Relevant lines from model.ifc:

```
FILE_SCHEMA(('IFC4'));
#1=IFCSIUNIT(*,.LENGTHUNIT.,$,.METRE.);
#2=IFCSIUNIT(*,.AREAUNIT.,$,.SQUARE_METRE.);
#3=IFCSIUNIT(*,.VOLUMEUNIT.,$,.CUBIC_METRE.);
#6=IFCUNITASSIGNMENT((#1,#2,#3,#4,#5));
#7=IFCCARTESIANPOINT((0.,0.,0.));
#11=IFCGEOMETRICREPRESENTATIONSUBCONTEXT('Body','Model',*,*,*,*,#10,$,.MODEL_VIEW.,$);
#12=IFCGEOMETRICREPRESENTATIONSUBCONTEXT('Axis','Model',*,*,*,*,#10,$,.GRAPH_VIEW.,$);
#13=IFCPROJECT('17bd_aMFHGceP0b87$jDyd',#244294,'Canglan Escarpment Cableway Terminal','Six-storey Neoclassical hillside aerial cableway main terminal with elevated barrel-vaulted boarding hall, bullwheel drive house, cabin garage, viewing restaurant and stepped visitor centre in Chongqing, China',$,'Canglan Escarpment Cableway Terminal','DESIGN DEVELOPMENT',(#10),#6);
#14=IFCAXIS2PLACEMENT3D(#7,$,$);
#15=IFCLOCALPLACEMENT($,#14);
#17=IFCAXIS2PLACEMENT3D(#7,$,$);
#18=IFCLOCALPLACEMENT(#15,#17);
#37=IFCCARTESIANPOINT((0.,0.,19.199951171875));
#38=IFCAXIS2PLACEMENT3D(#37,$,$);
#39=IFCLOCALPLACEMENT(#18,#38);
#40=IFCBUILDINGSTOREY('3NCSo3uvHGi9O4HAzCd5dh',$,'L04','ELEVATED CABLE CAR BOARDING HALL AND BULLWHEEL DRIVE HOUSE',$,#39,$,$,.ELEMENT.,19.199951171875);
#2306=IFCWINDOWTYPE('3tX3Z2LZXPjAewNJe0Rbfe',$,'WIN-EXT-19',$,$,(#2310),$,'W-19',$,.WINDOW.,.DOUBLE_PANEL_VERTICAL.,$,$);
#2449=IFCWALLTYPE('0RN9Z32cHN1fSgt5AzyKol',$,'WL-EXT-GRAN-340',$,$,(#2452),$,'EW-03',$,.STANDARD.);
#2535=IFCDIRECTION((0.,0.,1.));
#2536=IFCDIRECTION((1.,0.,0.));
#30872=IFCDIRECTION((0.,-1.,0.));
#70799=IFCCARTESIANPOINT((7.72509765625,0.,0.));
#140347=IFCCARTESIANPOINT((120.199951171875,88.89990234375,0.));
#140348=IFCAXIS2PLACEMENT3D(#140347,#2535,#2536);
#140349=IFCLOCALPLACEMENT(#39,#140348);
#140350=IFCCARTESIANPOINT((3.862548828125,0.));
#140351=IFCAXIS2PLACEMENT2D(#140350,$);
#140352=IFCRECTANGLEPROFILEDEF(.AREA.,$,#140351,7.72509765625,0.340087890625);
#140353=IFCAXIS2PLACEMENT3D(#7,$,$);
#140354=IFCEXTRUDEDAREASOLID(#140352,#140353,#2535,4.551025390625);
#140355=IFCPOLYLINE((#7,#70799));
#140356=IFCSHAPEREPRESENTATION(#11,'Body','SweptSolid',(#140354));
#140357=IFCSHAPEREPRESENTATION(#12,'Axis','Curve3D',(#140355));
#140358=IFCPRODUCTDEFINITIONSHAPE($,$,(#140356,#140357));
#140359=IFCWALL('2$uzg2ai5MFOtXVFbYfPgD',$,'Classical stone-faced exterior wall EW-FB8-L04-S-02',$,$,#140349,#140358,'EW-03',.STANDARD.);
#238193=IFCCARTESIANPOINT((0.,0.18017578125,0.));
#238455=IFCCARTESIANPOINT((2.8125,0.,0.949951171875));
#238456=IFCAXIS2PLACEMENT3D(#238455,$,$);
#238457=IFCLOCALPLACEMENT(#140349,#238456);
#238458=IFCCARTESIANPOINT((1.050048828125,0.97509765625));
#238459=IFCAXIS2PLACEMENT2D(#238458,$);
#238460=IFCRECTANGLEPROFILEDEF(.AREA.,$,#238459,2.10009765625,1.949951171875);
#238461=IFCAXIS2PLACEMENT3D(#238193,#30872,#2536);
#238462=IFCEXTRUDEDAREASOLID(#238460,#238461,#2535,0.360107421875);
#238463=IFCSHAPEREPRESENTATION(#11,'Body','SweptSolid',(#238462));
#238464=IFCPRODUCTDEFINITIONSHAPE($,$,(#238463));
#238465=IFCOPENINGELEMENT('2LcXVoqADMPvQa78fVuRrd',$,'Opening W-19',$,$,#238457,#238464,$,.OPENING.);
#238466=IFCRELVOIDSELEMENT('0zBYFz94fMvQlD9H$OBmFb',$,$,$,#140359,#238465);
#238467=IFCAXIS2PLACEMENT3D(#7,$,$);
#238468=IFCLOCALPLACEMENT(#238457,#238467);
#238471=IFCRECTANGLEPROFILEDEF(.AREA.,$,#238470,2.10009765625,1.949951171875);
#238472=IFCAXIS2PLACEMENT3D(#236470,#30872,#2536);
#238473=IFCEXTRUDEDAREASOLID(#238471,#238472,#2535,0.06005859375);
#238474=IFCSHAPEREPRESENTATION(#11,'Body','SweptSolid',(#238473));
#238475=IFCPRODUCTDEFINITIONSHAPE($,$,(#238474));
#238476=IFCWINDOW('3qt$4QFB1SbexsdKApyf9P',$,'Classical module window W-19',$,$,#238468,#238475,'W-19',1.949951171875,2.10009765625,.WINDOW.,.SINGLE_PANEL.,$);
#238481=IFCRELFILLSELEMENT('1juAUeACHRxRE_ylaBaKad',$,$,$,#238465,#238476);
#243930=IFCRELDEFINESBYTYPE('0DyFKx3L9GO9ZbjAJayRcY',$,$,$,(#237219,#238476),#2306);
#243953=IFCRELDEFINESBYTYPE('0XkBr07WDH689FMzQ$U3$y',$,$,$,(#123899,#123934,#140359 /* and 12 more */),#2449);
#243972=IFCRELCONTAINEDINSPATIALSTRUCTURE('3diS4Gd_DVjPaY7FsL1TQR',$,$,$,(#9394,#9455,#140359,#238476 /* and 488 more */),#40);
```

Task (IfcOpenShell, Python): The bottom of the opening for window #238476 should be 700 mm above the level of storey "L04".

```python
import numpy as np
import ifcopenshell
import ifcopenshell.api.geometry
import ifcopenshell.geom
import ifcopenshell.util.element
import ifcopenshell.util.placement
import ifcopenshell.util.shape
import ifcopenshell.util.unit

model = ifcopenshell.open("model.ifc")
unit_scale = ifcopenshell.util.unit.calculate_unit_scale(model)

window = model.by_id(238476)
opening = window.FillsVoids[0].RelatingOpeningElement
storey = ifcopenshell.util.element.get_container(window, ifc_class="IfcBuildingStorey")
level = ifcopenshell.util.placement.get_local_placement(storey.ObjectPlacement)[2, 3]

# The opening's origin need not be at the sill, so measure its lowest point.
shape = ifcopenshell.geom.create_shape(ifcopenshell.geom.settings(), opening)
bottom = ifcopenshell.util.shape.get_shape_bottom_elevation(shape, shape.geometry) / unit_scale
dz = level + 0.7 / unit_scale - bottom

shift = np.array([0.0, 0.0, dz])
# The window is placed relative to its opening, so it follows when the opening moves.
matrix = ifcopenshell.util.placement.get_local_placement(opening.ObjectPlacement)
matrix[:3, 3] += shift
ifcopenshell.api.geometry.edit_object_placement(
    model, product=opening, matrix=matrix, is_si=False, should_transform_children=True
)

print(f"moved by {dz * unit_scale:+.3f} m")

model.write("model_v2.ifc")
```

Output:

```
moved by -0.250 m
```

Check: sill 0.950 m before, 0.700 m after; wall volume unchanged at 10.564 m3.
